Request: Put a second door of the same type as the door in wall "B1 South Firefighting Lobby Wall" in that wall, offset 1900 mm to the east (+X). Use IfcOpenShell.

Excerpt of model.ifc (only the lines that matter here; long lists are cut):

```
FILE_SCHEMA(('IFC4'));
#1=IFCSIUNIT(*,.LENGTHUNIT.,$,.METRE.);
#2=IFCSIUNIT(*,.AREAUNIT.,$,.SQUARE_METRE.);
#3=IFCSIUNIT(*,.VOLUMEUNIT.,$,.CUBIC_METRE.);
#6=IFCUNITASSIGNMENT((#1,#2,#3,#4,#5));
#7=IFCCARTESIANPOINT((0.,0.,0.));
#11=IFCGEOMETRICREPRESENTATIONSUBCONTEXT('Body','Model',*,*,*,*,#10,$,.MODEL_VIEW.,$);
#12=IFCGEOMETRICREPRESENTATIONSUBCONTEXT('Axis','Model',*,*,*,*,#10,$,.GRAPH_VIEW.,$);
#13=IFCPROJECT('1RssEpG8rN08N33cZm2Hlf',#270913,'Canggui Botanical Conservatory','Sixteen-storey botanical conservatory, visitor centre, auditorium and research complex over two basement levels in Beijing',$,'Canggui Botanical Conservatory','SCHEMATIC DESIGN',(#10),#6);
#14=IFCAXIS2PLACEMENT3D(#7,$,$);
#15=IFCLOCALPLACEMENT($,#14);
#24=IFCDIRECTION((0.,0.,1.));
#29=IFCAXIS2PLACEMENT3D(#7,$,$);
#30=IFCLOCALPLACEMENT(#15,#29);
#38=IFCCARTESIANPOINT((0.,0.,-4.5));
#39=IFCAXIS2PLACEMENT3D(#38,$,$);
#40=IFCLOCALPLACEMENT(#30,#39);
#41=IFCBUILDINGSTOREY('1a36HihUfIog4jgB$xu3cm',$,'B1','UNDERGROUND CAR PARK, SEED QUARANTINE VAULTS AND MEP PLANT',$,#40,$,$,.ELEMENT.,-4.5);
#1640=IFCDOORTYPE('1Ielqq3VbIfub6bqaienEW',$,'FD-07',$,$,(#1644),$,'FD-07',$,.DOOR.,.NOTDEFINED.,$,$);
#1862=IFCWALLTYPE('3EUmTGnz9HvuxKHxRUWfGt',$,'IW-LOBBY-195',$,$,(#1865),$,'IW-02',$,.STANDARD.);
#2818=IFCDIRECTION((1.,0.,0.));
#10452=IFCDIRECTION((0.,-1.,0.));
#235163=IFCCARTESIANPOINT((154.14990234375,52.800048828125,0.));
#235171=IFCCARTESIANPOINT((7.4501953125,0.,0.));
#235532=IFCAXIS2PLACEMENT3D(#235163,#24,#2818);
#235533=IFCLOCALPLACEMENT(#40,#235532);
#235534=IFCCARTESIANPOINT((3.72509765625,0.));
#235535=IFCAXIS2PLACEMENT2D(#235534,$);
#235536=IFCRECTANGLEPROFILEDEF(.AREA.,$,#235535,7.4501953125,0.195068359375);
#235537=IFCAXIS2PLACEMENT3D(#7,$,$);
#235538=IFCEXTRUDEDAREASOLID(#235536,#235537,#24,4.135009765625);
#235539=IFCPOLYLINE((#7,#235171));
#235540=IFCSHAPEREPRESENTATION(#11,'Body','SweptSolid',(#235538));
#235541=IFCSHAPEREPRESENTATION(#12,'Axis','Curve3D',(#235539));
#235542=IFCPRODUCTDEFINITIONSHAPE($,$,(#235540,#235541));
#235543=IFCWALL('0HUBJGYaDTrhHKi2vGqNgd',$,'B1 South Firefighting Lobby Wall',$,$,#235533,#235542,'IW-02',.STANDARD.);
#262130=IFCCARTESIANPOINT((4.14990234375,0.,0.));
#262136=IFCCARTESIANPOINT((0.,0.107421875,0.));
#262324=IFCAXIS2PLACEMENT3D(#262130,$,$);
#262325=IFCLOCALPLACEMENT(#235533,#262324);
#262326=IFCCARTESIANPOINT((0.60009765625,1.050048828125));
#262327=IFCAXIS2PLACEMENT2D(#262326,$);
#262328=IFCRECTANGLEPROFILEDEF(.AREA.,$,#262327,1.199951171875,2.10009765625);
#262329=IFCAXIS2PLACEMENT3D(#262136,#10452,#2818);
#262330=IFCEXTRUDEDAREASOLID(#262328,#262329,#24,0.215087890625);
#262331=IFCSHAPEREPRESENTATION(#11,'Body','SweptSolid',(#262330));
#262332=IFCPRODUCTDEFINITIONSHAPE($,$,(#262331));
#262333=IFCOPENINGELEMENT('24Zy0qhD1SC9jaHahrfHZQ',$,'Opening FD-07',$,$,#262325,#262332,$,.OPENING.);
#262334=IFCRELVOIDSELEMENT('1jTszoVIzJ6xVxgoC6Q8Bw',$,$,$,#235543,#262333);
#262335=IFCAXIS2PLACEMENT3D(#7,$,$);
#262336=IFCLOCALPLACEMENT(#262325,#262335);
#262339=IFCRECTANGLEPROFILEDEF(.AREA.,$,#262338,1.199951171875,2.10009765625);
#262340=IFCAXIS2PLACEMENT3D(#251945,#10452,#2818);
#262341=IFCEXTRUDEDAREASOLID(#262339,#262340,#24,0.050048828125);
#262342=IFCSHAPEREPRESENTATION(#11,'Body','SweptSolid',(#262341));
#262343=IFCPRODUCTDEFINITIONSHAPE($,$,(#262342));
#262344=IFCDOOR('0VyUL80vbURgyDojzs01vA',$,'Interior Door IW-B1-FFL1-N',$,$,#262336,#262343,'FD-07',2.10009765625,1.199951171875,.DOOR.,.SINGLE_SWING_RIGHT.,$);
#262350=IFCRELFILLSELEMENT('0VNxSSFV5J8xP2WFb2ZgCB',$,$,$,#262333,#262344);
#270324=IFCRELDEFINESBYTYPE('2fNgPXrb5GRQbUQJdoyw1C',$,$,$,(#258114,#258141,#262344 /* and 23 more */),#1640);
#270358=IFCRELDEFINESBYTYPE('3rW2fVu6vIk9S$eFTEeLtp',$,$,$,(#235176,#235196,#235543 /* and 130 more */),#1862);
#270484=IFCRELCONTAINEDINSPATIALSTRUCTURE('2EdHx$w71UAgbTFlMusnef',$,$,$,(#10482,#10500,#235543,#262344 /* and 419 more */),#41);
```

```python
import ifcopenshell
import ifcopenshell.api.feature
import ifcopenshell.api.geometry
import ifcopenshell.api.root
import ifcopenshell.geom
import ifcopenshell.util.element
import ifcopenshell.util.placement
import ifcopenshell.util.shape

model = ifcopenshell.open("model.ifc")
settings = ifcopenshell.geom.settings()


def volume(element):
    """Net volume in cubic metres, openings subtracted."""
    shape = ifcopenshell.geom.create_shape(settings, element)
    return ifcopenshell.util.shape.get_volume(shape.geometry)


door = model.by_guid("0VyUL80vbURgyDojzs01vA")
opening = door.FillsVoids[0].RelatingOpeningElement
wall = opening.VoidsElements[0].RelatingBuildingElement
before = volume(wall)
shift = ifcopenshell.util.placement.get_local_placement(wall.ObjectPlacement)[:3, 0] * 1.9

# copy_class copies the void relationship, type, container and properties, but no geometry.
new_opening = ifcopenshell.api.root.copy_class(model, product=opening)
new_opening.Representation = ifcopenshell.util.element.copy_deep(
    model, opening.Representation, exclude=["IfcGeometricRepresentationContext", "IfcRepresentationMap"]
)
new_door = ifcopenshell.api.root.copy_class(model, product=door)
new_door.Representation = ifcopenshell.util.element.copy_deep(
    model, door.Representation, exclude=["IfcGeometricRepresentationContext", "IfcRepresentationMap"]
)
new_door.Tag = None
ifcopenshell.api.feature.add_filling(model, opening=new_opening, element=new_door)

for old, new in ((opening, new_opening), (door, new_door)):
    matrix = ifcopenshell.util.placement.get_local_placement(old.ObjectPlacement)
    matrix[:3, 3] += shift
    ifcopenshell.api.geometry.edit_object_placement(model, product=new, matrix=matrix, is_si=False)

after = volume(wall)

print(f"wall volume {before:.3f} -> {after:.3f} m3")

model.write("model-out.ifc")
```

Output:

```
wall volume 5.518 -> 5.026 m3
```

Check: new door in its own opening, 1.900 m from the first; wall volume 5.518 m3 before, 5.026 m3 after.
